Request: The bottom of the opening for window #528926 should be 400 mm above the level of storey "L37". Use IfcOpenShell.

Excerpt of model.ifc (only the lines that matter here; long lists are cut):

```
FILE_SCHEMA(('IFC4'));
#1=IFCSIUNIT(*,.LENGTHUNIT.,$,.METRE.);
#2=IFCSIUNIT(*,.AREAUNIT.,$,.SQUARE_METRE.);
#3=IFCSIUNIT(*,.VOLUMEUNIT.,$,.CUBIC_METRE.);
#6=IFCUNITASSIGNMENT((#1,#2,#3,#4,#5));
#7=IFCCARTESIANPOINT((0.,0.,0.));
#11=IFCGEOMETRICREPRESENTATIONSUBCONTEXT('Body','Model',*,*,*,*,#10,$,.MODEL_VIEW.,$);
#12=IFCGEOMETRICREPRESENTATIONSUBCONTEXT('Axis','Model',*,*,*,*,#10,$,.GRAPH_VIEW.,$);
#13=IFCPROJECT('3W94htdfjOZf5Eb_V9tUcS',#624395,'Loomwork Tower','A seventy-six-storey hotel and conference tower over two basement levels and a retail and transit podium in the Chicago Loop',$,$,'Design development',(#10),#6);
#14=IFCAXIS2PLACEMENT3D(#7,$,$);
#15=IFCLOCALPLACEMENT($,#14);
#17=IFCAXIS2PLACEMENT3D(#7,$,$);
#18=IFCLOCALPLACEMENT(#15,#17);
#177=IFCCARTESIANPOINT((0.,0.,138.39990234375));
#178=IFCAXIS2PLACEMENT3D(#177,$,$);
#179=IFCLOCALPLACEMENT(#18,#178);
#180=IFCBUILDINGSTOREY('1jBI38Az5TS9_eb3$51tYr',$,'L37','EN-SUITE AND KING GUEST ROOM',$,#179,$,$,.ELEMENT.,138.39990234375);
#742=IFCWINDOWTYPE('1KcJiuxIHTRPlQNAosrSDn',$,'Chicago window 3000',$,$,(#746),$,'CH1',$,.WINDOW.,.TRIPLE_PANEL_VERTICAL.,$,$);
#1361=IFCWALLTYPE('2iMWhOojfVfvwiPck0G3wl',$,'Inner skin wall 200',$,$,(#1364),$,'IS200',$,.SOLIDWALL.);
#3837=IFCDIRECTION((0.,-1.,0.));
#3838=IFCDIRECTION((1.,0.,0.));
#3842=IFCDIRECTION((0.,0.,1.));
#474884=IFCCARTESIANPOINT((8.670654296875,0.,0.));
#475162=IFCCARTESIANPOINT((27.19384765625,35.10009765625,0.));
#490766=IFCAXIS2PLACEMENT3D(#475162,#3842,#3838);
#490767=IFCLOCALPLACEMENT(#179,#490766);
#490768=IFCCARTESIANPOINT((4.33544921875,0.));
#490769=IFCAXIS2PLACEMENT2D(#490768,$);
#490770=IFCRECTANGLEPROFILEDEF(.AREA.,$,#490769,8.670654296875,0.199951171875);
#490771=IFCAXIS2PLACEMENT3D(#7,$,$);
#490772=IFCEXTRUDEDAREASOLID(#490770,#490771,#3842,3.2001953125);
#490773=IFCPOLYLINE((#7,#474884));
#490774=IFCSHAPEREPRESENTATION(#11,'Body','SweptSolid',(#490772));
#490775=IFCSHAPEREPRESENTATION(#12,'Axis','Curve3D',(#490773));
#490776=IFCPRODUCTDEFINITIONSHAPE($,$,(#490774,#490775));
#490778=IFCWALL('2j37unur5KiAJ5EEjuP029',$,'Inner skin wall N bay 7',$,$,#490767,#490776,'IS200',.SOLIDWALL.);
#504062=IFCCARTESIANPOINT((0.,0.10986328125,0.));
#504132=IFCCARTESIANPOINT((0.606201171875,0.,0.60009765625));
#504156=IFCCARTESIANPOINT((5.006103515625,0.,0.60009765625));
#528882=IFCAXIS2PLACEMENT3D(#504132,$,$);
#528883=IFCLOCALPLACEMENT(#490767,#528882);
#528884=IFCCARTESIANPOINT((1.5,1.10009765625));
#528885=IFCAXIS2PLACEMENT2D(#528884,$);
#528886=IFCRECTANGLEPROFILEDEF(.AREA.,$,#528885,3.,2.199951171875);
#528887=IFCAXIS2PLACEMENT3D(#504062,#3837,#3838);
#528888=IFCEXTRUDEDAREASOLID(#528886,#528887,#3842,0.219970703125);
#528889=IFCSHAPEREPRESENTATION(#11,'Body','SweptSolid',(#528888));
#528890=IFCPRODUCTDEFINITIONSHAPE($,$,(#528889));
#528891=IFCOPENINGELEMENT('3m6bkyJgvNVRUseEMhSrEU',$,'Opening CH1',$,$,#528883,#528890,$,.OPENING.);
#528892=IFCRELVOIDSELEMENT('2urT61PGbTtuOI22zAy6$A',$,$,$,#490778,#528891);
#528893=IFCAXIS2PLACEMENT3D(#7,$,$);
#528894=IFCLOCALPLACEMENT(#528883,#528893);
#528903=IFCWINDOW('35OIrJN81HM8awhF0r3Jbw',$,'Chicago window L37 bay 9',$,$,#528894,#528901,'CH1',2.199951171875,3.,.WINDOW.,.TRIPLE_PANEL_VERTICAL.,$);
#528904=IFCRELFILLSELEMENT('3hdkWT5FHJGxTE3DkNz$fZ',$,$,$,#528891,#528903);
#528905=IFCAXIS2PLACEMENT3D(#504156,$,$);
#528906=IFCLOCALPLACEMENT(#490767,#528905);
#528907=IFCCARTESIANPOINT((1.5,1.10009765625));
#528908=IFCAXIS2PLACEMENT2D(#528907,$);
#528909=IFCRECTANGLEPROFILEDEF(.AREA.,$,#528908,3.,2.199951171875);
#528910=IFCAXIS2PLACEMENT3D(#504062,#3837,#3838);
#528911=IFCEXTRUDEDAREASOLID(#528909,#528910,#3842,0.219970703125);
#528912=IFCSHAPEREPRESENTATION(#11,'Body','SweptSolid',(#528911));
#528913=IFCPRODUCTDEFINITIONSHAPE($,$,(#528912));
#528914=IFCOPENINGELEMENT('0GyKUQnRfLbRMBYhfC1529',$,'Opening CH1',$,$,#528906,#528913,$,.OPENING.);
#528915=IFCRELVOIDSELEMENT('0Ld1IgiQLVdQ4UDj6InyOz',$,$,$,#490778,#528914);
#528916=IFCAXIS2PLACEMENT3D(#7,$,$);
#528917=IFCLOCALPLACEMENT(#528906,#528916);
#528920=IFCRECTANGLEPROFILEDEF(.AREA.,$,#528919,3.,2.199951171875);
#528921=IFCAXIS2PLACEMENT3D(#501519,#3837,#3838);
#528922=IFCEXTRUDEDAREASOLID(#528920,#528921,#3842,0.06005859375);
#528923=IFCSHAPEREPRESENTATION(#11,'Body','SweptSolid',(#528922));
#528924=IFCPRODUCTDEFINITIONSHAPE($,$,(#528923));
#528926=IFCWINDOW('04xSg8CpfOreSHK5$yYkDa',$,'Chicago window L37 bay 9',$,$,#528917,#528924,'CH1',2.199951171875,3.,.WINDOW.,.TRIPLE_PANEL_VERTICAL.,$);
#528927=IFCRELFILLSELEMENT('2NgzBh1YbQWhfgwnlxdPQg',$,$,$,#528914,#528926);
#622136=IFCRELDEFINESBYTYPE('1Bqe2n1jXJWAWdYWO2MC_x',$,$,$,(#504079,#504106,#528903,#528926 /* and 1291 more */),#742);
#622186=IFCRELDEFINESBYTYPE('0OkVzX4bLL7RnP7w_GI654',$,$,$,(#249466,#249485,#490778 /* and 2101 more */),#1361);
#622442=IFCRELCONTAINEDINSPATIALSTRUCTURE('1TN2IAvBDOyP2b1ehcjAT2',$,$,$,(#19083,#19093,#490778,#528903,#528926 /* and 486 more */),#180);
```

```python
import numpy as np
import ifcopenshell
import ifcopenshell.api.geometry
import ifcopenshell.geom
import ifcopenshell.util.element
import ifcopenshell.util.placement
import ifcopenshell.util.shape
import ifcopenshell.util.unit

model = ifcopenshell.open("model.ifc")
unit_scale = ifcopenshell.util.unit.calculate_unit_scale(model)

window = model.by_guid("04xSg8CpfOreSHK5$yYkDa")
opening = window.FillsVoids[0].RelatingOpeningElement
storey = ifcopenshell.util.element.get_container(window, ifc_class="IfcBuildingStorey")
level = ifcopenshell.util.placement.get_local_placement(storey.ObjectPlacement)[2, 3]

# The opening's origin need not be at the sill, so measure its lowest point.
shape = ifcopenshell.geom.create_shape(ifcopenshell.geom.settings(), opening)
bottom = ifcopenshell.util.shape.get_shape_bottom_elevation(shape, shape.geometry) / unit_scale
dz = level + 0.4 / unit_scale - bottom

shift = np.array([0.0, 0.0, dz])
# The window is placed relative to its opening, so it follows when the opening moves.
matrix = ifcopenshell.util.placement.get_local_placement(opening.ObjectPlacement)
matrix[:3, 3] += shift
ifcopenshell.api.geometry.edit_object_placement(
    model, product=opening, matrix=matrix, is_si=False, should_transform_children=True
)

print(f"moved by {dz * unit_scale:+.3f} m")

model.write("model_rev.ifc")
```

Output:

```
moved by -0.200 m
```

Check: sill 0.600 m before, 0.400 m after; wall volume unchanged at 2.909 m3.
